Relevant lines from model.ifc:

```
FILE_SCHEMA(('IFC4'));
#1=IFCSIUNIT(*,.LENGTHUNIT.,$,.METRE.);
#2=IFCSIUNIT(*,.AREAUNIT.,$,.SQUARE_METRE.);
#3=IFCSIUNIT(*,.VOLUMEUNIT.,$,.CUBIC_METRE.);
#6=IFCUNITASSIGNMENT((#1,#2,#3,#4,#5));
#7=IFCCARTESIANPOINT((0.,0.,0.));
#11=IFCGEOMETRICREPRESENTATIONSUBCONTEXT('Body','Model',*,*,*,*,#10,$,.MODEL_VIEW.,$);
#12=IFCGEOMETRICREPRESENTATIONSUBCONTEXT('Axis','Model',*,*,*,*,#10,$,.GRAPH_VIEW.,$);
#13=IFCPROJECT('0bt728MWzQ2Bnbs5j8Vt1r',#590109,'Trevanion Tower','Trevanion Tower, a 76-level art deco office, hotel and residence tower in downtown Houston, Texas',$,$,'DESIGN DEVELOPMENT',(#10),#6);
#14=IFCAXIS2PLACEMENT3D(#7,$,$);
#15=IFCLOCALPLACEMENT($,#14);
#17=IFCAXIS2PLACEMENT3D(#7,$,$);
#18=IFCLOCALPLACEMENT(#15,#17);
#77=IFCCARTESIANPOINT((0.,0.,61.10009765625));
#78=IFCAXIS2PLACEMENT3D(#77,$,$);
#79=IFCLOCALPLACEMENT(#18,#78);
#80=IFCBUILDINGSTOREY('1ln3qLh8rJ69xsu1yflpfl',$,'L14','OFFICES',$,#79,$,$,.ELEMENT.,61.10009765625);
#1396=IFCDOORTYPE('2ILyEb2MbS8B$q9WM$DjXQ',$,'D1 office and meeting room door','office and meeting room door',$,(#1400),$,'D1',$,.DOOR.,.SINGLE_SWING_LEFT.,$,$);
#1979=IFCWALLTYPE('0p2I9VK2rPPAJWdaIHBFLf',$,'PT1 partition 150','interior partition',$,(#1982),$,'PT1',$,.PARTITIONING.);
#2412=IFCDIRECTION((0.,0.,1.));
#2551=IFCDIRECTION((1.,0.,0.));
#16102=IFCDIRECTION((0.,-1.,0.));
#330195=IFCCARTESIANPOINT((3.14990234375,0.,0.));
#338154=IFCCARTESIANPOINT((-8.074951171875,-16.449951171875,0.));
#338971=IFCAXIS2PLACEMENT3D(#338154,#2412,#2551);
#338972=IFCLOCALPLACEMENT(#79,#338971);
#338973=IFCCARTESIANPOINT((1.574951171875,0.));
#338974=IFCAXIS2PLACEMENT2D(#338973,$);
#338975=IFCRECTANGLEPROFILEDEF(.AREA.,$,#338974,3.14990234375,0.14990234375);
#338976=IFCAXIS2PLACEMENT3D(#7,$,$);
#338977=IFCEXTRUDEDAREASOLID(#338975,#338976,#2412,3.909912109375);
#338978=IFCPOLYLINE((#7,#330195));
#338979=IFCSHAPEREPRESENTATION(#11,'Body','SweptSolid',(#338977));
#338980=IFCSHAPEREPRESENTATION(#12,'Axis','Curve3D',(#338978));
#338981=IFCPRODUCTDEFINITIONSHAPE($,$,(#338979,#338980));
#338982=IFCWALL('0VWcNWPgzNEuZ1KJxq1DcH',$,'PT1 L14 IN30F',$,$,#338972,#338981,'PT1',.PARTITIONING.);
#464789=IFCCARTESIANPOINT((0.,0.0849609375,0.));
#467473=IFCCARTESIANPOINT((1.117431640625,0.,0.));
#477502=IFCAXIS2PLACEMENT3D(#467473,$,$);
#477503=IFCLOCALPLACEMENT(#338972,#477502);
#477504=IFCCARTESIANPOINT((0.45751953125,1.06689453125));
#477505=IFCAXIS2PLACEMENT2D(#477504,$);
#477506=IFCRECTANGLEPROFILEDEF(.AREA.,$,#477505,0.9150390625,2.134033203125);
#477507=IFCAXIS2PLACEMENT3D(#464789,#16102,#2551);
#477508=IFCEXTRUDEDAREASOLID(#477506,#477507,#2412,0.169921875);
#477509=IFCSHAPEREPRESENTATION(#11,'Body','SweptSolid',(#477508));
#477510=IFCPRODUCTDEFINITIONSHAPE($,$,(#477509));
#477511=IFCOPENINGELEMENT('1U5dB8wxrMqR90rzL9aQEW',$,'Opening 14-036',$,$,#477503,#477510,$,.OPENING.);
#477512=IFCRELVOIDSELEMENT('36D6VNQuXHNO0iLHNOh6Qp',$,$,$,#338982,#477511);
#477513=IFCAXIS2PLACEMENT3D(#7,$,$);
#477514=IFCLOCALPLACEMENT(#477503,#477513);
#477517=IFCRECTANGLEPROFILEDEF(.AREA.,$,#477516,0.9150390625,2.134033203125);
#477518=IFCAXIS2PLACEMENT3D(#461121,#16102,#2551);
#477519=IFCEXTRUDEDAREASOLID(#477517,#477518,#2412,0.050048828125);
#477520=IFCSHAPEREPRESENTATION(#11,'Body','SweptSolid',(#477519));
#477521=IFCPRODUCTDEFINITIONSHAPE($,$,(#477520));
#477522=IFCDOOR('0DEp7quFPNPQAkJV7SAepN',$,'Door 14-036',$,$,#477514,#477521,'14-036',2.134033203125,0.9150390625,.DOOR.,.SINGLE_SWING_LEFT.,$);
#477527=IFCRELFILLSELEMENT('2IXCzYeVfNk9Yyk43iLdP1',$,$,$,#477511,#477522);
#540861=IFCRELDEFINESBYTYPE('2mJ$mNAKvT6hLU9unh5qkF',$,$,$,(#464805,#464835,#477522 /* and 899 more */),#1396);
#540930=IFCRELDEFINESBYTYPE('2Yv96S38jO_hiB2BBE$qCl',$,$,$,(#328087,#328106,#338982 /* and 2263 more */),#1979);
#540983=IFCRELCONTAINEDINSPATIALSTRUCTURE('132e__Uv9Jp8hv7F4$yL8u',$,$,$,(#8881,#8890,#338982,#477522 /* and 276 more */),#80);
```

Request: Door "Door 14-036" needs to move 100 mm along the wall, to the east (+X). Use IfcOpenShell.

```python
import ifcopenshell
import ifcopenshell.api.geometry
import ifcopenshell.util.placement
import ifcopenshell.util.unit

model = ifcopenshell.open("model.ifc")
unit_scale = ifcopenshell.util.unit.calculate_unit_scale(model)

door = model.by_guid("0DEp7quFPNPQAkJV7SAepN")
opening = door.FillsVoids[0].RelatingOpeningElement
wall = opening.VoidsElements[0].RelatingBuildingElement

wall_matrix = ifcopenshell.util.placement.get_local_placement(wall.ObjectPlacement)
shift = wall_matrix[:3, 0] * 0.1 / unit_scale
before = ifcopenshell.util.placement.get_local_placement(door.ObjectPlacement)[:3, 3].copy()

# The door is placed relative to its opening, so it follows when the opening moves.
matrix = ifcopenshell.util.placement.get_local_placement(opening.ObjectPlacement)
matrix[:3, 3] += shift
ifcopenshell.api.geometry.edit_object_placement(
    model, product=opening, matrix=matrix, is_si=False, should_transform_children=True
)

after = ifcopenshell.util.placement.get_local_placement(door.ObjectPlacement)[:3, 3]
print("door moved by", (after - before).round(3) + 0.0)

model.write("model_edited.ifc")
```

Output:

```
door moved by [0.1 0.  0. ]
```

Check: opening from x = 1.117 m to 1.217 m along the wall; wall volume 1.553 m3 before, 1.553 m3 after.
